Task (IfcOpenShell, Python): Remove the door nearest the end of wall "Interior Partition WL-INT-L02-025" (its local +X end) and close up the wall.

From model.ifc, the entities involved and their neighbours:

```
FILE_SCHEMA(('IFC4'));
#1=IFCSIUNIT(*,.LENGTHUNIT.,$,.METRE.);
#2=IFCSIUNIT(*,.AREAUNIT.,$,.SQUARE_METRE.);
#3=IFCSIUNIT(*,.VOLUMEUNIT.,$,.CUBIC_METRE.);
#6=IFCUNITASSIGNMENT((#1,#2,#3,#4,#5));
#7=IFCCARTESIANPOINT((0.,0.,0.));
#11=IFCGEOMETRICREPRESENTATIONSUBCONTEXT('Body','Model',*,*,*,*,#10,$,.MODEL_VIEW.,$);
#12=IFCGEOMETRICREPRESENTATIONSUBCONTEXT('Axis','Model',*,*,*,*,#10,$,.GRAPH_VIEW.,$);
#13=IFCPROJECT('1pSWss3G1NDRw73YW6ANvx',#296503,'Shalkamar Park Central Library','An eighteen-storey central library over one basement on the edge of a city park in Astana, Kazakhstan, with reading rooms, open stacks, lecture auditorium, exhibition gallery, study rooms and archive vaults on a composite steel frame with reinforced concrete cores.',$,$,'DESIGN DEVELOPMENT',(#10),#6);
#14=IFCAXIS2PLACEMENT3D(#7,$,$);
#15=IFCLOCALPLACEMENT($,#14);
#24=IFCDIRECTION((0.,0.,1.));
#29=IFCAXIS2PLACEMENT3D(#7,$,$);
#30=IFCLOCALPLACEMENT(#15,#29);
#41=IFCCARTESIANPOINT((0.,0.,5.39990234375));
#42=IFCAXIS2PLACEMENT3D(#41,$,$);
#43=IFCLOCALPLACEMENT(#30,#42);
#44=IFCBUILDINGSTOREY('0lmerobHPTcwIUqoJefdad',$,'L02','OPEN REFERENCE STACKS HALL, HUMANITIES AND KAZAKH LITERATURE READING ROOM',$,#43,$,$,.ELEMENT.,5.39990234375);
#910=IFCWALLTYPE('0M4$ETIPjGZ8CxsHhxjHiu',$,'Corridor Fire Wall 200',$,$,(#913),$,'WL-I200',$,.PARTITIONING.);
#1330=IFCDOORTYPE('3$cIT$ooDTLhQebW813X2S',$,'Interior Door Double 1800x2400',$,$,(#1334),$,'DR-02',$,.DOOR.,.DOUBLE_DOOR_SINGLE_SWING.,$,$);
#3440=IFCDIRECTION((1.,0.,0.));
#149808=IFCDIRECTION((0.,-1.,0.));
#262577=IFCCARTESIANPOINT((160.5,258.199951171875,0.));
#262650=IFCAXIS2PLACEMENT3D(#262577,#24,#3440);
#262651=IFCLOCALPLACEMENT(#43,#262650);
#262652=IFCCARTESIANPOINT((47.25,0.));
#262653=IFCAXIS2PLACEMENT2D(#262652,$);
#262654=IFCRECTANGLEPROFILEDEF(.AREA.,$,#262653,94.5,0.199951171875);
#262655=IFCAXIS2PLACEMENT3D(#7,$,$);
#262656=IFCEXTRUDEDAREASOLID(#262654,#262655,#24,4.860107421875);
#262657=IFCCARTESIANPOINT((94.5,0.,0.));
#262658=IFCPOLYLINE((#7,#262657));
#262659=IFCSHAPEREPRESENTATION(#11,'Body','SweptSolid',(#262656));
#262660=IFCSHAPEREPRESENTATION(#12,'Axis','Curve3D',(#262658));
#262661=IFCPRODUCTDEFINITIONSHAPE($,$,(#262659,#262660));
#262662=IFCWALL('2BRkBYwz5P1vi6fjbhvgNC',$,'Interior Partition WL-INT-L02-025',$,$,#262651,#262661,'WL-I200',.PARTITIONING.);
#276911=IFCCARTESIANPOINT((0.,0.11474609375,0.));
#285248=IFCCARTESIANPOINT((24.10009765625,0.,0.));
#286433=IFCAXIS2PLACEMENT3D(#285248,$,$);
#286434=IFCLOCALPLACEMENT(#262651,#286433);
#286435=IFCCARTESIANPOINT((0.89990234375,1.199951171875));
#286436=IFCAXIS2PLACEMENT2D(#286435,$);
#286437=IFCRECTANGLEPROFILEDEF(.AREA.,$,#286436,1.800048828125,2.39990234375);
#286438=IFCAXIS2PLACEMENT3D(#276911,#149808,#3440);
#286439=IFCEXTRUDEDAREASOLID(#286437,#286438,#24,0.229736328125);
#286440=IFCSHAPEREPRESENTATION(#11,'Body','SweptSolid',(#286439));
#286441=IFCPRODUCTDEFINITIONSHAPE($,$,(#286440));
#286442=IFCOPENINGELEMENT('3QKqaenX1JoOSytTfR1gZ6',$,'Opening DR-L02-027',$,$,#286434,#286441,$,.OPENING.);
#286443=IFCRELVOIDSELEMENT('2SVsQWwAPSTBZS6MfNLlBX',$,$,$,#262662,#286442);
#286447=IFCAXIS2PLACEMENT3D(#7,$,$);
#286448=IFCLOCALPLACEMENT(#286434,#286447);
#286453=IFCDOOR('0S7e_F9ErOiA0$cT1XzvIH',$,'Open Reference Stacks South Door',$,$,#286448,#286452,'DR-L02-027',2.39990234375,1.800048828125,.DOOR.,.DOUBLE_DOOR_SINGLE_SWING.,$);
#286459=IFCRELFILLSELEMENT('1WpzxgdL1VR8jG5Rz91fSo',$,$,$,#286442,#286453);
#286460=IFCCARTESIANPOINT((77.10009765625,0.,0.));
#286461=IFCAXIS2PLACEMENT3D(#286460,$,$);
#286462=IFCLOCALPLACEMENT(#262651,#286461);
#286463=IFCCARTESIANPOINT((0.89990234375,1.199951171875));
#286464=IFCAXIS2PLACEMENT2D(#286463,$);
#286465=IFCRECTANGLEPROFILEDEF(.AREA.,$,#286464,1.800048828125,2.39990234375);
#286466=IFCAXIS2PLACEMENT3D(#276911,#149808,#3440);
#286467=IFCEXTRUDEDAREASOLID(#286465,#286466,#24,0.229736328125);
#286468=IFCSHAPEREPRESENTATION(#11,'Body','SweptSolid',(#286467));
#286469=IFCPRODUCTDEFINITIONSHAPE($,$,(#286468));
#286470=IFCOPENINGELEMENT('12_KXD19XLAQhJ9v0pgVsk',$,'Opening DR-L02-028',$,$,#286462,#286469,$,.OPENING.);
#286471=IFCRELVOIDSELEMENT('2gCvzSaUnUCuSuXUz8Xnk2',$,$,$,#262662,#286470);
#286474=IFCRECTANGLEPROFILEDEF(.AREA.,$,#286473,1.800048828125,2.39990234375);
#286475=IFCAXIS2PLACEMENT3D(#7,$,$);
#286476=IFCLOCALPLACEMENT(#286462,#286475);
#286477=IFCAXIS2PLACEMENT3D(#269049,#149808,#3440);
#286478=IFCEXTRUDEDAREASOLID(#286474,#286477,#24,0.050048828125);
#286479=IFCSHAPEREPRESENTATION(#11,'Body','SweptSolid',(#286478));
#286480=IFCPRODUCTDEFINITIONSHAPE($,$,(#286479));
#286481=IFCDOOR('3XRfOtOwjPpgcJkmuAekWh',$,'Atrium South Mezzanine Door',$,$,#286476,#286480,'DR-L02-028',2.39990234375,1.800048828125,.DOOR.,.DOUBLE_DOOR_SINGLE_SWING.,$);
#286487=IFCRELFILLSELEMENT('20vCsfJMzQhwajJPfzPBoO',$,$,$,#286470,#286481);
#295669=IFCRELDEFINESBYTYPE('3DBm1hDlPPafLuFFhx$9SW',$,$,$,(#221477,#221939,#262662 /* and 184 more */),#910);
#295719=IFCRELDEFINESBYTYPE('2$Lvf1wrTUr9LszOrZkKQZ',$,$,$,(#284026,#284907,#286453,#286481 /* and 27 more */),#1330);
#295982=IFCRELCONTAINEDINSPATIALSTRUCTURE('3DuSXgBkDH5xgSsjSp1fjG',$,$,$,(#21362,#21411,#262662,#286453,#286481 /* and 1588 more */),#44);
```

```python
import ifcopenshell
import ifcopenshell.api.feature
import ifcopenshell.api.root
import ifcopenshell.geom
import ifcopenshell.util.shape

model = ifcopenshell.open("model.ifc")
settings = ifcopenshell.geom.settings()


def volume(element):
    """Net volume in cubic metres, openings subtracted."""
    shape = ifcopenshell.geom.create_shape(settings, element)
    return ifcopenshell.util.shape.get_volume(shape.geometry)


door = model.by_guid("3XRfOtOwjPpgcJkmuAekWh")
opening = door.FillsVoids[0].RelatingOpeningElement
wall = opening.VoidsElements[0].RelatingBuildingElement
before = volume(wall)

ifcopenshell.api.root.remove_product(model, product=door)
ifcopenshell.api.feature.remove_feature(model, feature=opening)

after = volume(wall)

print(f"wall volume {before:.3f} -> {after:.3f} m3")

model.write("model-out.ifc")
```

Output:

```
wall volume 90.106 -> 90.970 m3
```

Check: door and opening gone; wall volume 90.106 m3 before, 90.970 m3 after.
